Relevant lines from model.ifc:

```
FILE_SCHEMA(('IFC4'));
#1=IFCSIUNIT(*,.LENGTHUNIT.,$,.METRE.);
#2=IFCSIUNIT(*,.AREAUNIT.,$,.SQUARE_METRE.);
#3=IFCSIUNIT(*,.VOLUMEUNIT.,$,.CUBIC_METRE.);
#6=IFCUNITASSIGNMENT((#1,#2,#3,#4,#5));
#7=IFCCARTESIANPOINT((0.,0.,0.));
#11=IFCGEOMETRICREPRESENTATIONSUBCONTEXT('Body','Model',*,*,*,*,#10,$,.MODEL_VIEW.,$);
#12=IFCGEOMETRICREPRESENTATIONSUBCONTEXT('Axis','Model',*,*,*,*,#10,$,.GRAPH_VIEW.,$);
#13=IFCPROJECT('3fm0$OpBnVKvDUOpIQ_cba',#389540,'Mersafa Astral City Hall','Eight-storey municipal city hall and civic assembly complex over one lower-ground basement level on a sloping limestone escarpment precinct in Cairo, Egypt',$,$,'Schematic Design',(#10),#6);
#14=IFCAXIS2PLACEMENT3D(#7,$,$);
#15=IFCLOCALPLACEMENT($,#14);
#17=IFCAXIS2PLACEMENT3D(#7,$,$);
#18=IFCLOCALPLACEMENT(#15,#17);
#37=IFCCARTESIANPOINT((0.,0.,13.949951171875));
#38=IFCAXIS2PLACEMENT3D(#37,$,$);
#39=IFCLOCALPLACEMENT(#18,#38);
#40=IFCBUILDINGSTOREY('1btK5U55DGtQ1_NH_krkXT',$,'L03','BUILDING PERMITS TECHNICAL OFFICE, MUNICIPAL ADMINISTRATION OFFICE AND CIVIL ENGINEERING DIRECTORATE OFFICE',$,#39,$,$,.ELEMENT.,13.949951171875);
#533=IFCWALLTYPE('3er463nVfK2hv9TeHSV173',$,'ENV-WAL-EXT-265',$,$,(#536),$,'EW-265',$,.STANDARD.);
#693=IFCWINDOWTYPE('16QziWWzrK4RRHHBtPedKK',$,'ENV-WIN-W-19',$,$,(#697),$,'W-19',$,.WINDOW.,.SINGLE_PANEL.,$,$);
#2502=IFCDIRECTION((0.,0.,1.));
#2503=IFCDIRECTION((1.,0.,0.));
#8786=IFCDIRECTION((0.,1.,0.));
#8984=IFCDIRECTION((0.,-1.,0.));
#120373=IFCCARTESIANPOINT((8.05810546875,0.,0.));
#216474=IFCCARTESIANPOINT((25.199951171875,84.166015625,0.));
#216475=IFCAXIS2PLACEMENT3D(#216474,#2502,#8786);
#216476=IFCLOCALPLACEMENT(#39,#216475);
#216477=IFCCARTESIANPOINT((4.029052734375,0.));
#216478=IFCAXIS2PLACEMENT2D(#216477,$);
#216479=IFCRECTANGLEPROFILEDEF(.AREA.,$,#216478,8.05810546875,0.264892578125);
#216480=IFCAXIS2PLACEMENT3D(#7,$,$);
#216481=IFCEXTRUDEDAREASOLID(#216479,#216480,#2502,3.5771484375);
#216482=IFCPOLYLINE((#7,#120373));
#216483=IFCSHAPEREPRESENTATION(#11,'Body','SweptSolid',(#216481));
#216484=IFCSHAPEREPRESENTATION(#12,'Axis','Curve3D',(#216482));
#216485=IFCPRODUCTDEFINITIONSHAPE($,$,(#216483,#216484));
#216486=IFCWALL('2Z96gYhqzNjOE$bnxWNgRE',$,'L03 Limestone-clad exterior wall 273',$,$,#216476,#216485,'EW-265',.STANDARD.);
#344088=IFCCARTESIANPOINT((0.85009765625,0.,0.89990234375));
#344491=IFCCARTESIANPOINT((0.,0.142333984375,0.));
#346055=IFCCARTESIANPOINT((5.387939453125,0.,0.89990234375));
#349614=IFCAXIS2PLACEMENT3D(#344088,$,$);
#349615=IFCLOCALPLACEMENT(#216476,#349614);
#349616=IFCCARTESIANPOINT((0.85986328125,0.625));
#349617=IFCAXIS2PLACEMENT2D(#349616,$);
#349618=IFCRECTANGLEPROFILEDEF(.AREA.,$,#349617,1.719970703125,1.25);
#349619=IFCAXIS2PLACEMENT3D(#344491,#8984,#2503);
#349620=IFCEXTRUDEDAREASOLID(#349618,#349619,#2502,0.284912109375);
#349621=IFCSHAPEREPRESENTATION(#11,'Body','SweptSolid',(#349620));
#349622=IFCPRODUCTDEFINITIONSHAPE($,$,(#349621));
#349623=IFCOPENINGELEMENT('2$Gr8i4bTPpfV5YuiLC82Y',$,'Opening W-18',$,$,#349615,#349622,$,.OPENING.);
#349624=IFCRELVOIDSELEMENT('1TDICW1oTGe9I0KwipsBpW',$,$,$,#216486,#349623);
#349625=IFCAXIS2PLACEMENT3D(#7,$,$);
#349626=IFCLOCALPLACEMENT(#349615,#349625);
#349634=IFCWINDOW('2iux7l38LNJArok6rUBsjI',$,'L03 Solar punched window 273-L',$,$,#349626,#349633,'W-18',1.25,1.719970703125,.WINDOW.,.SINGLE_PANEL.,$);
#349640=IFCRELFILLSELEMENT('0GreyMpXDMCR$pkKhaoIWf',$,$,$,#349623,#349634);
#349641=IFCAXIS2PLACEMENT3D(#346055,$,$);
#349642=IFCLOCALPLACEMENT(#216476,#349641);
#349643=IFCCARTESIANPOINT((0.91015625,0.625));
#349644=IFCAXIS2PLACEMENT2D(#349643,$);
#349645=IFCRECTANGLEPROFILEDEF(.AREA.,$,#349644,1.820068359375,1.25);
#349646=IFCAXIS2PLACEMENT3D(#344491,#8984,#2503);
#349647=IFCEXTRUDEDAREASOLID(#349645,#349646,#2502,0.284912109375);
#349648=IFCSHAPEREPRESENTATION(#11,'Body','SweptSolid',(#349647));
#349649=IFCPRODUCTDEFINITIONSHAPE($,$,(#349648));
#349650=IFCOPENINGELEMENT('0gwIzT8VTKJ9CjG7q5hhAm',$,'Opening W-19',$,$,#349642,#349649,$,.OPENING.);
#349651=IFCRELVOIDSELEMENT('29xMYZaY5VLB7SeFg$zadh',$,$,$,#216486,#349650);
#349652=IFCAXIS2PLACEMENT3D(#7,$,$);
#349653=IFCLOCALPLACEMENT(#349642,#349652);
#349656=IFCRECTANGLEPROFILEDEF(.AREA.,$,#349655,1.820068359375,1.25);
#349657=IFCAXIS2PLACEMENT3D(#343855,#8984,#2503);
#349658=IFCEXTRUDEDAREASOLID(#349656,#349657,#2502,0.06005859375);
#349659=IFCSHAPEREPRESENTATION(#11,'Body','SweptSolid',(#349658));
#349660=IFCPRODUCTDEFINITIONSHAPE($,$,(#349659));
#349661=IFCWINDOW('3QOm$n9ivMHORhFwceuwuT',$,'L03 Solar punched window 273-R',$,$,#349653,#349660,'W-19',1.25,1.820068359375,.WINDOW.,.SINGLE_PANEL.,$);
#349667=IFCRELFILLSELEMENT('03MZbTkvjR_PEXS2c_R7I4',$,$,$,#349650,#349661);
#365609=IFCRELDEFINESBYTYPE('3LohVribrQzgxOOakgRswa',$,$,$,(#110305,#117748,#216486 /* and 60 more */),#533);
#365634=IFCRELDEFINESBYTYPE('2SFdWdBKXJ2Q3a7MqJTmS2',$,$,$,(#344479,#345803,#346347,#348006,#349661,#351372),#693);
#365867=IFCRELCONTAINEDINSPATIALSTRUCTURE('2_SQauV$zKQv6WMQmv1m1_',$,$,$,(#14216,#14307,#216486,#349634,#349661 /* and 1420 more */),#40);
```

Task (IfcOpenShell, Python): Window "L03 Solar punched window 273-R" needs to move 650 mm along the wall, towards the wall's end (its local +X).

```python
import ifcopenshell
import ifcopenshell.api.geometry
import ifcopenshell.util.placement

model = ifcopenshell.open("model.ifc")

window = model.by_guid("3QOm$n9ivMHORhFwceuwuT")
opening = window.FillsVoids[0].RelatingOpeningElement
wall = opening.VoidsElements[0].RelatingBuildingElement

wall_matrix = ifcopenshell.util.placement.get_local_placement(wall.ObjectPlacement)
shift = wall_matrix[:3, 0] * 0.65
before = ifcopenshell.util.placement.get_local_placement(window.ObjectPlacement)[:3, 3].copy()

# The window is placed relative to its opening, so it follows when the opening moves.
matrix = ifcopenshell.util.placement.get_local_placement(opening.ObjectPlacement)
matrix[:3, 3] += shift
ifcopenshell.api.geometry.edit_object_placement(
    model, product=opening, matrix=matrix, is_si=False, should_transform_children=True
)

after = ifcopenshell.util.placement.get_local_placement(window.ObjectPlacement)[:3, 3]
print("window moved by", (after - before).round(3) + 0.0)

model.write("model-out.ifc")
```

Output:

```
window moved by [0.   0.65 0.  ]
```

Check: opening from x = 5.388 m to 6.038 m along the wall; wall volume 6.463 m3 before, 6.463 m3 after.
